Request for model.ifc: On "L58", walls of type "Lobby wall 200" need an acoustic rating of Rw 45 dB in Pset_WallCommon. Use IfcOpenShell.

First a look at what the model holds.

```python
import ifcopenshell
import ifcopenshell.util.element

model = ifcopenshell.open("model.ifc")
print(model.schema)
storey = next(s for s in model.by_type("IfcBuildingStorey") if s.Name == "L58")
walls = [e for e in ifcopenshell.util.element.get_decomposition(storey) if e.is_a("IfcWall")]
seen = {}
for e in walls:
    element_type = ifcopenshell.util.element.get_type(e)
    key = (element_type.Name if element_type != e and element_type else None, ifcopenshell.util.element.get_pset(e, "Pset_WallCommon", "AcousticRating"))
    seen[key] = seen.get(key, 0) + 1
for (name, value), count in sorted(seen.items(), key=str):
    print(count, "x", name, "|", value)
```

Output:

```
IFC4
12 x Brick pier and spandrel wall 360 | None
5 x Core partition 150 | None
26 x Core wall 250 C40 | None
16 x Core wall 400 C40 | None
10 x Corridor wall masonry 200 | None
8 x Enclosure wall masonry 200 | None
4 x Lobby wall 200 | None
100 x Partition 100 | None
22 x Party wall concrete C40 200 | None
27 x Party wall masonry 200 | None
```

```python
import ifcopenshell
import ifcopenshell.api.pset
import ifcopenshell.util.element

model = ifcopenshell.open("model.ifc")

storey = next(s for s in model.by_type("IfcBuildingStorey") if s.Name == "L58")
walls = [e for e in ifcopenshell.util.element.get_decomposition(storey) if e.is_a("IfcWall")]

count = 0
for e in walls:
    element_type = ifcopenshell.util.element.get_type(e)
    if element_type in (None, e) or element_type.Name != "Lobby wall 200":
        continue
    found = ifcopenshell.util.element.get_pset(e, "Pset_WallCommon", should_inherit=False)
    if found:
        pset = model.by_id(found["id"])
        if len(ifcopenshell.util.element.get_elements_by_pset(pset)) > 1:
            pset = ifcopenshell.api.pset.unshare_pset(model, products=[e], pset=pset)[0]
    else:
        pset = ifcopenshell.api.pset.add_pset(model, product=e, name="Pset_WallCommon")
    ifcopenshell.api.pset.edit_pset(model, pset=pset, properties={"AcousticRating": "Rw 45 dB"})
    count += 1

print(count, "walls updated")

model.write("model_edited.ifc")
```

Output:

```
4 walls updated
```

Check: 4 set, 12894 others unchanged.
